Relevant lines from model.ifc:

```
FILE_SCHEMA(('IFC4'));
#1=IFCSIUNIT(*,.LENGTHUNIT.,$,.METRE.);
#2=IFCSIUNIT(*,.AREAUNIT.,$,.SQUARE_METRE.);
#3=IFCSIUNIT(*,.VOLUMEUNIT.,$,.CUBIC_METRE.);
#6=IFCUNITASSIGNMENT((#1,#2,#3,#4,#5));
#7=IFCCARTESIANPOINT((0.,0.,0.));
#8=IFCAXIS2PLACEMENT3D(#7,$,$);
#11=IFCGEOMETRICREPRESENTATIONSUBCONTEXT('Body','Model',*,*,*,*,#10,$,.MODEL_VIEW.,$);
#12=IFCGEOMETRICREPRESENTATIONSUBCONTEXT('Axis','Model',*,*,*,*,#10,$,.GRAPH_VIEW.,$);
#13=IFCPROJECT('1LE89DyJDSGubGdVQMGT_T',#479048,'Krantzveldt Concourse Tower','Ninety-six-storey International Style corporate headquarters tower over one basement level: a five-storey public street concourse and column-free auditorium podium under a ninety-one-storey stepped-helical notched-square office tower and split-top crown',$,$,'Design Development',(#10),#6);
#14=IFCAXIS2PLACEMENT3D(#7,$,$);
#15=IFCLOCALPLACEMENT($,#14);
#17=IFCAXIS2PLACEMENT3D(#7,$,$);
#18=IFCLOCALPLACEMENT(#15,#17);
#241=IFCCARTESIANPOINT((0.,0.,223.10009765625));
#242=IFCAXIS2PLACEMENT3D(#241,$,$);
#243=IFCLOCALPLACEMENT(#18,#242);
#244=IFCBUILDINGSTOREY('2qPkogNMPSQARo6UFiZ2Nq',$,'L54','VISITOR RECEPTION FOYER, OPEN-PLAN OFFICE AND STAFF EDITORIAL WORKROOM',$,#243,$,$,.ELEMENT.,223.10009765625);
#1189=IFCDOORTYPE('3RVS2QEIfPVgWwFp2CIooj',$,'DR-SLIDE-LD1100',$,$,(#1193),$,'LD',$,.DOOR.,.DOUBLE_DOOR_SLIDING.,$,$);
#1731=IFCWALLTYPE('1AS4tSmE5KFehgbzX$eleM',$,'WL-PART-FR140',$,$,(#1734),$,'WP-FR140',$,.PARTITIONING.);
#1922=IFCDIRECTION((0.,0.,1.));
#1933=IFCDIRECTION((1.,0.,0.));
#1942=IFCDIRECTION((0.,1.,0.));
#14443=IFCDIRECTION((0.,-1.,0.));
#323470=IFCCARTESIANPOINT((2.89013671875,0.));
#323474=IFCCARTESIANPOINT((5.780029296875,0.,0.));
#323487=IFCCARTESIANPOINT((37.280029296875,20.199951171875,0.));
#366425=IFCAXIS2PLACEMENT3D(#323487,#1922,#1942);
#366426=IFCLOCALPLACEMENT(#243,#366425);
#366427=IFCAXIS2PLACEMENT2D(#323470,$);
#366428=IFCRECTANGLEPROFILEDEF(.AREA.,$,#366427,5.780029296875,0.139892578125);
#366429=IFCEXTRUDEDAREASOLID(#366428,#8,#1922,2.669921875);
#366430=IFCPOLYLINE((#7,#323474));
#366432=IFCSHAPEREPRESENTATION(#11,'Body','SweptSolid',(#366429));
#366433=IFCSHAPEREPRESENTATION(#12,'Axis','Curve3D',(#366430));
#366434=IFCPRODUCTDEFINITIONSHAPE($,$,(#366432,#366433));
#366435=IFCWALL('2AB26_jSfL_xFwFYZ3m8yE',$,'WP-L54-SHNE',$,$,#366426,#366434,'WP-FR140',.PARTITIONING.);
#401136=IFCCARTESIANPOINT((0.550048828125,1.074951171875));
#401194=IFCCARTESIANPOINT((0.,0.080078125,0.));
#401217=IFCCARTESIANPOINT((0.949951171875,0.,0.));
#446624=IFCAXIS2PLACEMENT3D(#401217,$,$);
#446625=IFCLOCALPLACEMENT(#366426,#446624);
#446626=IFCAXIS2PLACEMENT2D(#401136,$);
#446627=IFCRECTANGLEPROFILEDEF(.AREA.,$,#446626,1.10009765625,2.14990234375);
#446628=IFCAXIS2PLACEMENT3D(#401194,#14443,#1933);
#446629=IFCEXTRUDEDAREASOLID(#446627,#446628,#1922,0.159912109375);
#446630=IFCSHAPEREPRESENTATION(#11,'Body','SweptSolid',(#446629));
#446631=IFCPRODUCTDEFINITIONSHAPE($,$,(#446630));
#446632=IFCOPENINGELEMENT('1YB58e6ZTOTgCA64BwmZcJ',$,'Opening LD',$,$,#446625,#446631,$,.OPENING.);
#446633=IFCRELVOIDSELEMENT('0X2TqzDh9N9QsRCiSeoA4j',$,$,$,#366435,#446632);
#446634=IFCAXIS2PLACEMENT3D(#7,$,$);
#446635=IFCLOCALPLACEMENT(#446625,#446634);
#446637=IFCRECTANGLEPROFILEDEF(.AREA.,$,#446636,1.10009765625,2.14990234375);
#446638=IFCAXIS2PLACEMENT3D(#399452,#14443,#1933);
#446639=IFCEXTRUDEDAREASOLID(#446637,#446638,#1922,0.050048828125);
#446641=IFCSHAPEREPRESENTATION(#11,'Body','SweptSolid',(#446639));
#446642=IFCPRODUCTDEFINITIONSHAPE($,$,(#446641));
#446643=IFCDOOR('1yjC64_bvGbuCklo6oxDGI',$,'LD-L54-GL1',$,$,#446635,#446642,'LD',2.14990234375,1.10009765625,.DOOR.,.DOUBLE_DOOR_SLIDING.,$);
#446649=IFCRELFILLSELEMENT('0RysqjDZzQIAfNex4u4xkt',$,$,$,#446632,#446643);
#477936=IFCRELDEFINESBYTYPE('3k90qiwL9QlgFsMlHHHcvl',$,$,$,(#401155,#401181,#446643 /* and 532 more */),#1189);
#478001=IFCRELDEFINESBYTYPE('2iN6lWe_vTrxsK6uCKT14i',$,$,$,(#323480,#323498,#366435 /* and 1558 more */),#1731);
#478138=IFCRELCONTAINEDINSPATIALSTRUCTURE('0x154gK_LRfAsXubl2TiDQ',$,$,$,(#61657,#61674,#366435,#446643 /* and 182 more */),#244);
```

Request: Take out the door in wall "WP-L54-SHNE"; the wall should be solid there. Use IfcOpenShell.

```python
import ifcopenshell
import ifcopenshell.api.feature
import ifcopenshell.api.root
import ifcopenshell.geom
import ifcopenshell.util.shape

model = ifcopenshell.open("model.ifc")
settings = ifcopenshell.geom.settings()


def volume(element):
    """Net volume in cubic metres, openings subtracted."""
    shape = ifcopenshell.geom.create_shape(settings, element)
    return ifcopenshell.util.shape.get_volume(shape.geometry)


door = model.by_id(446643)
opening = door.FillsVoids[0].RelatingOpeningElement
wall = opening.VoidsElements[0].RelatingBuildingElement
before = volume(wall)

ifcopenshell.api.root.remove_product(model, product=door)
ifcopenshell.api.feature.remove_feature(model, feature=opening)

after = volume(wall)

print(f"wall volume {before:.3f} -> {after:.3f} m3")

model.write("model_edited.ifc")
```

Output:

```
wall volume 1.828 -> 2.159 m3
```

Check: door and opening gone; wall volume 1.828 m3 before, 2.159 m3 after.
